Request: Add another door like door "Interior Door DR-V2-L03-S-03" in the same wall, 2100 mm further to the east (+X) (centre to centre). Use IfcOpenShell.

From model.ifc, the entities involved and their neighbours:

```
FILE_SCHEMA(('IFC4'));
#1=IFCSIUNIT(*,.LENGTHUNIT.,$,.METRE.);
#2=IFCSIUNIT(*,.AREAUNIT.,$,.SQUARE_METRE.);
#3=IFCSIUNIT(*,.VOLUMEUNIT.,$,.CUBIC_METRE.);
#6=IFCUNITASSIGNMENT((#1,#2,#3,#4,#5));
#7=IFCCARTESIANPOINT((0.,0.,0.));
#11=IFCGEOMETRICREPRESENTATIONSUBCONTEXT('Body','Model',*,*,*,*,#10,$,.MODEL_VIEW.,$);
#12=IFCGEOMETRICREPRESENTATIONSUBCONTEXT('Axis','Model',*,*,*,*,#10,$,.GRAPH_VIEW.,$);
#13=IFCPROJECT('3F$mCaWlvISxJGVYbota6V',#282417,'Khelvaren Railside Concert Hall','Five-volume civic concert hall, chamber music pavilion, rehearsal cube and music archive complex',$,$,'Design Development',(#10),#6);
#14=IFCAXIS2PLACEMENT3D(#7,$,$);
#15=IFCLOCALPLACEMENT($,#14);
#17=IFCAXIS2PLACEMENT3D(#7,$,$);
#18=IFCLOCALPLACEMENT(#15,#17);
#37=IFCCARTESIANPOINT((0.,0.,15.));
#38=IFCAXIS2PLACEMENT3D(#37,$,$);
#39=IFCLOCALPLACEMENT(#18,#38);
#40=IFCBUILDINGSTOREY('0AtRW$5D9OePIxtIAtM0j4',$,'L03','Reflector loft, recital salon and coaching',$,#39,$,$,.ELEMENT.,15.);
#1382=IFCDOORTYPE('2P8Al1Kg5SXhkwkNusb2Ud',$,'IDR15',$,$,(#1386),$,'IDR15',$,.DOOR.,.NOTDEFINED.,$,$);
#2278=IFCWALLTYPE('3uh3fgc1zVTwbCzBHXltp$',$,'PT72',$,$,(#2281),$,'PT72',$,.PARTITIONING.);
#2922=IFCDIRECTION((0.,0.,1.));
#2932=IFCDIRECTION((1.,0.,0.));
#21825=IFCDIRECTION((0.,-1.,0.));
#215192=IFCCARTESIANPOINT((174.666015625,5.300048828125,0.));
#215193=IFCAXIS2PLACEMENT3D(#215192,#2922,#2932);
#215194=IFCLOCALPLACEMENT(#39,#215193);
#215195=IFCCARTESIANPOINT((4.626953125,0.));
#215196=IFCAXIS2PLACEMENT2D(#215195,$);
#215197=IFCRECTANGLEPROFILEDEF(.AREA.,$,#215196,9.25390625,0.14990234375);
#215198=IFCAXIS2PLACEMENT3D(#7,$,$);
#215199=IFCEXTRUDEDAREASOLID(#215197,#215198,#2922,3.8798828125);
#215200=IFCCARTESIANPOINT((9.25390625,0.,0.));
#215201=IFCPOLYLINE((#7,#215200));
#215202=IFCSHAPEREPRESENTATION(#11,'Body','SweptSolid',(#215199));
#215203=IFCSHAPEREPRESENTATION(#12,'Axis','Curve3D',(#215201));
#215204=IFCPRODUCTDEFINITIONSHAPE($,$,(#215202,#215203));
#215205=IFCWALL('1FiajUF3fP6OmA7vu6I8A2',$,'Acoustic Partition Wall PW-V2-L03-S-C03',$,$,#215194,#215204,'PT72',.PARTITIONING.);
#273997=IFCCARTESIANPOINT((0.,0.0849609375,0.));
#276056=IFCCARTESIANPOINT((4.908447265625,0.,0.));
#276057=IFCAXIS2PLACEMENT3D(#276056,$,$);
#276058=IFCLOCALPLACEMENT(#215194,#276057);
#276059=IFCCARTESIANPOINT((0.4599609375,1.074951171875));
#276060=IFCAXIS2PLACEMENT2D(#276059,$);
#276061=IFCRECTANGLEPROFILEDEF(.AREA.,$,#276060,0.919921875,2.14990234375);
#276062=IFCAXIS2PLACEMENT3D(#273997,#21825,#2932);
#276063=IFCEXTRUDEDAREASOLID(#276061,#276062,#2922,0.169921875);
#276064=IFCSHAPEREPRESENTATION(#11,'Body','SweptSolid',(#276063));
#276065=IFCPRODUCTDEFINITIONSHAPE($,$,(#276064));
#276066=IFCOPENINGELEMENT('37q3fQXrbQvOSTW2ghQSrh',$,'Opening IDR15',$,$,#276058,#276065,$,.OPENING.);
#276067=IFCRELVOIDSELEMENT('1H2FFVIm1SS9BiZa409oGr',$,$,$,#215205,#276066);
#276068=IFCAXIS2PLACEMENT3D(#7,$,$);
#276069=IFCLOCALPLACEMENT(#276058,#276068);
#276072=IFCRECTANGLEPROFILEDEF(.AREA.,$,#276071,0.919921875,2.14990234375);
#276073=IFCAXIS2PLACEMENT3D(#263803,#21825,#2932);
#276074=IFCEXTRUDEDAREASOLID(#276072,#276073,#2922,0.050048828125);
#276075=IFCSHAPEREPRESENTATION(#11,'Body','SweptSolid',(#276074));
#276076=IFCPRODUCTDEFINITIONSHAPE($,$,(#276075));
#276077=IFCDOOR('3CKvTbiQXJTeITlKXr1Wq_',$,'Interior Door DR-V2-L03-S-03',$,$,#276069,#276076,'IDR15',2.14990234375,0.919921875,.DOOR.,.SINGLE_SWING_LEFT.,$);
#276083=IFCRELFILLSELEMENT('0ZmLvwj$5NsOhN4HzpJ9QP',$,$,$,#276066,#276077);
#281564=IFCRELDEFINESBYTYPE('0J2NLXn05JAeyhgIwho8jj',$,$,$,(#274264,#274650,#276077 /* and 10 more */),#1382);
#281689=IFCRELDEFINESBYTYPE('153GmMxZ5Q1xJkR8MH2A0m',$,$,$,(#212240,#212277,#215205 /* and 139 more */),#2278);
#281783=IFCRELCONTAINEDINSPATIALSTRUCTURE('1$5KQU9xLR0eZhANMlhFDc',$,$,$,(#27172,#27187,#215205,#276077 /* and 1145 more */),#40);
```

```python
import ifcopenshell
import ifcopenshell.api.feature
import ifcopenshell.api.geometry
import ifcopenshell.api.root
import ifcopenshell.geom
import ifcopenshell.util.element
import ifcopenshell.util.placement
import ifcopenshell.util.shape
import ifcopenshell.util.unit

model = ifcopenshell.open("model.ifc")
unit_scale = ifcopenshell.util.unit.calculate_unit_scale(model)
settings = ifcopenshell.geom.settings()


def volume(element):
    """Net volume in cubic metres, openings subtracted."""
    shape = ifcopenshell.geom.create_shape(settings, element)
    return ifcopenshell.util.shape.get_volume(shape.geometry)


door = model.by_guid("3CKvTbiQXJTeITlKXr1Wq_")
opening = door.FillsVoids[0].RelatingOpeningElement
wall = opening.VoidsElements[0].RelatingBuildingElement
before = volume(wall)
shift = ifcopenshell.util.placement.get_local_placement(wall.ObjectPlacement)[:3, 0] * 2.1 / unit_scale

# copy_class copies the void relationship, type, container and properties, but no geometry.
new_opening = ifcopenshell.api.root.copy_class(model, product=opening)
new_opening.Representation = ifcopenshell.util.element.copy_deep(
    model, opening.Representation, exclude=["IfcGeometricRepresentationContext", "IfcRepresentationMap"]
)
new_door = ifcopenshell.api.root.copy_class(model, product=door)
new_door.Representation = ifcopenshell.util.element.copy_deep(
    model, door.Representation, exclude=["IfcGeometricRepresentationContext", "IfcRepresentationMap"]
)
new_door.Tag = None
ifcopenshell.api.feature.add_filling(model, opening=new_opening, element=new_door)

for old, new in ((opening, new_opening), (door, new_door)):
    matrix = ifcopenshell.util.placement.get_local_placement(old.ObjectPlacement)
    matrix[:3, 3] += shift
    ifcopenshell.api.geometry.edit_object_placement(model, product=new, matrix=matrix, is_si=False)

after = volume(wall)

print(f"wall volume {before:.3f} -> {after:.3f} m3")

model.write("model_rev.ifc")
```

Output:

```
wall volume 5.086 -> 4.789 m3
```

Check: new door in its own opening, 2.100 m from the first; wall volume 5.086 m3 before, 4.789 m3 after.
